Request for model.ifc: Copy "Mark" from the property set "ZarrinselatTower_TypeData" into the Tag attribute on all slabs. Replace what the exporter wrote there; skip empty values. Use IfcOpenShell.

First a look at what the model holds.

```python
import ifcopenshell
import ifcopenshell.util.element

model = ifcopenshell.open("model.ifc")
print(model.schema)
slabs = model.by_type("IfcSlab")
print(len(slabs), "slabs")
for e in slabs[:8]:
    source = ifcopenshell.util.element.get_pset(e, "ZarrinselatTower_TypeData", "Mark")
    target = e.Tag
    print(e.id(), repr(source), repr(target), sep=" | ")
```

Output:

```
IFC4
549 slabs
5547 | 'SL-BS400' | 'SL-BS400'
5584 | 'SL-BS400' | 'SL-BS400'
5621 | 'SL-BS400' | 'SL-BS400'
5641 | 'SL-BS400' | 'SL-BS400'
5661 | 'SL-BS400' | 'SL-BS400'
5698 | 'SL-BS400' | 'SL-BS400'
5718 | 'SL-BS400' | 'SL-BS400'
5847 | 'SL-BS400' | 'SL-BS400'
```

```python
import ifcopenshell
import ifcopenshell.util.element

model = ifcopenshell.open("model.ifc")

count = 0
for e in model.by_type("IfcSlab"):
    value = ifcopenshell.util.element.get_pset(e, "ZarrinselatTower_TypeData", "Mark")
    current = e.Tag
    if not value or not value.strip() or current == value:
        continue
    e.Tag = value
    count += 1

print(count, "slabs updated")

model.write("model_updated.ifc")
```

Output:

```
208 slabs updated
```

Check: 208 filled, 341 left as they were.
